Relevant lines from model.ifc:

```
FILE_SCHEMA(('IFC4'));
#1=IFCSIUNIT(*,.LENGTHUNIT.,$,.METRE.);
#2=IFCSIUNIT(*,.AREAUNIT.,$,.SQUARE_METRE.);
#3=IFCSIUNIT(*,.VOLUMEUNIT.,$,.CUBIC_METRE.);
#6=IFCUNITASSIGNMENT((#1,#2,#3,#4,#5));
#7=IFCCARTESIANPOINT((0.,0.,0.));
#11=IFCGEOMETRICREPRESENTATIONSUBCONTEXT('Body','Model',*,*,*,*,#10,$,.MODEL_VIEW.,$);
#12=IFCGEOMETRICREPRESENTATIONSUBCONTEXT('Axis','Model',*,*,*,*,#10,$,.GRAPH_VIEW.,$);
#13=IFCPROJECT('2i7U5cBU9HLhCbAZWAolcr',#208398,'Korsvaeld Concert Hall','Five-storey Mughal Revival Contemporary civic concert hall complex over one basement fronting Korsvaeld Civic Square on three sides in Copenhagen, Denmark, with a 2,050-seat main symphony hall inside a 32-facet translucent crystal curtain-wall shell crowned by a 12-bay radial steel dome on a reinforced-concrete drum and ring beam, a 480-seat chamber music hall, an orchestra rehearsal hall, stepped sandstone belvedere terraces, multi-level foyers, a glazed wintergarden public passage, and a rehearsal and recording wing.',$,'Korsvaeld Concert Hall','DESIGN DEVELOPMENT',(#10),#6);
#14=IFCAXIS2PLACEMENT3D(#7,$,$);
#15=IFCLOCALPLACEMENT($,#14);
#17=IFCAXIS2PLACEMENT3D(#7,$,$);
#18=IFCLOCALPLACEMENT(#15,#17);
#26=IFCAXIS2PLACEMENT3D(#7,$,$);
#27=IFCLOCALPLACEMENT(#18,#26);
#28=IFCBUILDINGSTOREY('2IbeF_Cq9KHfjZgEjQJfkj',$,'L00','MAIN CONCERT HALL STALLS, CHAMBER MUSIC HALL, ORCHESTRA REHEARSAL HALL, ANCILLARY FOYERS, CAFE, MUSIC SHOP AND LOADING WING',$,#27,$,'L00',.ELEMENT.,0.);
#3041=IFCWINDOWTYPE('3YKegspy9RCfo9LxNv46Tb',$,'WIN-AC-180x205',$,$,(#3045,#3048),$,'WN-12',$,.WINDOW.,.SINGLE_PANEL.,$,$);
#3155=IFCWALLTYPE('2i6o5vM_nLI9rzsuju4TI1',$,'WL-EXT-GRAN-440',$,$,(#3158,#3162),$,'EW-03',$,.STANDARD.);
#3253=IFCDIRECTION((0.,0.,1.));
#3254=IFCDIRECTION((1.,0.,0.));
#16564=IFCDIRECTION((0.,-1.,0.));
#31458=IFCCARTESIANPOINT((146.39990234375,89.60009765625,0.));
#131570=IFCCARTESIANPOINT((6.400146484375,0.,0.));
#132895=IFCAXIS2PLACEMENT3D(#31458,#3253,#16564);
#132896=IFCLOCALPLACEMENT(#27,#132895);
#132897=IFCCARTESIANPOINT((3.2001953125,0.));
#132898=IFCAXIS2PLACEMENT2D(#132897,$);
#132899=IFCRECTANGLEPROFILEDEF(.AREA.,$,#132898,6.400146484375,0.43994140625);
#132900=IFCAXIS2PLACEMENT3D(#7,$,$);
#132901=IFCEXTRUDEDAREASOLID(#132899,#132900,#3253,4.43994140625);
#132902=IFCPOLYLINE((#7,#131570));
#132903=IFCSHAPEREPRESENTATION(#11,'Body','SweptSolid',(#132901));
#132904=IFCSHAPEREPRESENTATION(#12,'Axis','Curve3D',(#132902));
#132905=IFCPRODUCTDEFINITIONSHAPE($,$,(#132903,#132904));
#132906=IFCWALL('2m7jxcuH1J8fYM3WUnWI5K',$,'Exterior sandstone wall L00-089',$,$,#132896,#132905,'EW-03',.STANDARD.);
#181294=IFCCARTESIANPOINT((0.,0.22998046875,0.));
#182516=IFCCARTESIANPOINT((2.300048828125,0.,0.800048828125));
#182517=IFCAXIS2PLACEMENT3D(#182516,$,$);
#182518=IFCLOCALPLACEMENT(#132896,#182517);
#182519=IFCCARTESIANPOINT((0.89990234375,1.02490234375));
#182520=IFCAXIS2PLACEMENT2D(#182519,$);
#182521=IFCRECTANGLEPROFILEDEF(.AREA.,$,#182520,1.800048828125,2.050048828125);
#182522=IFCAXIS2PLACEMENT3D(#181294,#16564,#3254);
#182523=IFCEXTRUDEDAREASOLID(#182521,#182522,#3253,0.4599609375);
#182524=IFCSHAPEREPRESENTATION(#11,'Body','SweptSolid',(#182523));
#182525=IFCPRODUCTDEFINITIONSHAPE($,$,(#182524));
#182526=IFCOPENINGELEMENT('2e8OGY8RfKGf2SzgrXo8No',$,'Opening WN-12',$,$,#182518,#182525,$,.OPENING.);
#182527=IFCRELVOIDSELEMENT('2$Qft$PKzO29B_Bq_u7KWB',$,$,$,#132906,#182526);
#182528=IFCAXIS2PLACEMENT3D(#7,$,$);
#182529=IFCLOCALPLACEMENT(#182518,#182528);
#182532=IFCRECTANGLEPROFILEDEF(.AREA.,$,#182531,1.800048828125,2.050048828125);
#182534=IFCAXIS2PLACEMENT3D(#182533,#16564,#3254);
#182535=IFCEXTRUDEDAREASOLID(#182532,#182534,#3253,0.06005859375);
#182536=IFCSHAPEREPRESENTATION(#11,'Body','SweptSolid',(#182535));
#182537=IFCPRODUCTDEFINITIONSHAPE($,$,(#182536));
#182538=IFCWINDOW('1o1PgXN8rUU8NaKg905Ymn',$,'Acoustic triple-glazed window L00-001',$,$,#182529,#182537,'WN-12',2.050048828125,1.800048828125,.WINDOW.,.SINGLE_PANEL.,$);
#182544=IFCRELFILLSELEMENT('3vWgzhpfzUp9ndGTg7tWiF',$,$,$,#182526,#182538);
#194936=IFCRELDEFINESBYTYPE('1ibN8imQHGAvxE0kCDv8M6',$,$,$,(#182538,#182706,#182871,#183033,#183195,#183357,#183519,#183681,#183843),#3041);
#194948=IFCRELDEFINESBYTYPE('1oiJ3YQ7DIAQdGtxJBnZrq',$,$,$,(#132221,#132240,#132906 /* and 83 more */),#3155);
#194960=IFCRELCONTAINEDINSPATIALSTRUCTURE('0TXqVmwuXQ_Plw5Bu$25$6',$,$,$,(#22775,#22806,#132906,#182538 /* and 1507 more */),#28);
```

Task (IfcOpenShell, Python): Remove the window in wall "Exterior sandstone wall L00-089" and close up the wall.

```python
import ifcopenshell
import ifcopenshell.api.feature
import ifcopenshell.api.root
import ifcopenshell.geom
import ifcopenshell.util.shape

model = ifcopenshell.open("model.ifc")
settings = ifcopenshell.geom.settings()


def volume(element):
    """Net volume in cubic metres, openings subtracted."""
    shape = ifcopenshell.geom.create_shape(settings, element)
    return ifcopenshell.util.shape.get_volume(shape.geometry)


window = model.by_guid("1o1PgXN8rUU8NaKg905Ymn")
opening = window.FillsVoids[0].RelatingOpeningElement
wall = opening.VoidsElements[0].RelatingBuildingElement
before = volume(wall)

ifcopenshell.api.root.remove_product(model, product=window)
ifcopenshell.api.feature.remove_feature(model, feature=opening)

after = volume(wall)

print(f"wall volume {before:.3f} -> {after:.3f} m3")

model.write("model-out.ifc")
```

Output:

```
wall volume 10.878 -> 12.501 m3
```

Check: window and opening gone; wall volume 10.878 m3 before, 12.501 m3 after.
